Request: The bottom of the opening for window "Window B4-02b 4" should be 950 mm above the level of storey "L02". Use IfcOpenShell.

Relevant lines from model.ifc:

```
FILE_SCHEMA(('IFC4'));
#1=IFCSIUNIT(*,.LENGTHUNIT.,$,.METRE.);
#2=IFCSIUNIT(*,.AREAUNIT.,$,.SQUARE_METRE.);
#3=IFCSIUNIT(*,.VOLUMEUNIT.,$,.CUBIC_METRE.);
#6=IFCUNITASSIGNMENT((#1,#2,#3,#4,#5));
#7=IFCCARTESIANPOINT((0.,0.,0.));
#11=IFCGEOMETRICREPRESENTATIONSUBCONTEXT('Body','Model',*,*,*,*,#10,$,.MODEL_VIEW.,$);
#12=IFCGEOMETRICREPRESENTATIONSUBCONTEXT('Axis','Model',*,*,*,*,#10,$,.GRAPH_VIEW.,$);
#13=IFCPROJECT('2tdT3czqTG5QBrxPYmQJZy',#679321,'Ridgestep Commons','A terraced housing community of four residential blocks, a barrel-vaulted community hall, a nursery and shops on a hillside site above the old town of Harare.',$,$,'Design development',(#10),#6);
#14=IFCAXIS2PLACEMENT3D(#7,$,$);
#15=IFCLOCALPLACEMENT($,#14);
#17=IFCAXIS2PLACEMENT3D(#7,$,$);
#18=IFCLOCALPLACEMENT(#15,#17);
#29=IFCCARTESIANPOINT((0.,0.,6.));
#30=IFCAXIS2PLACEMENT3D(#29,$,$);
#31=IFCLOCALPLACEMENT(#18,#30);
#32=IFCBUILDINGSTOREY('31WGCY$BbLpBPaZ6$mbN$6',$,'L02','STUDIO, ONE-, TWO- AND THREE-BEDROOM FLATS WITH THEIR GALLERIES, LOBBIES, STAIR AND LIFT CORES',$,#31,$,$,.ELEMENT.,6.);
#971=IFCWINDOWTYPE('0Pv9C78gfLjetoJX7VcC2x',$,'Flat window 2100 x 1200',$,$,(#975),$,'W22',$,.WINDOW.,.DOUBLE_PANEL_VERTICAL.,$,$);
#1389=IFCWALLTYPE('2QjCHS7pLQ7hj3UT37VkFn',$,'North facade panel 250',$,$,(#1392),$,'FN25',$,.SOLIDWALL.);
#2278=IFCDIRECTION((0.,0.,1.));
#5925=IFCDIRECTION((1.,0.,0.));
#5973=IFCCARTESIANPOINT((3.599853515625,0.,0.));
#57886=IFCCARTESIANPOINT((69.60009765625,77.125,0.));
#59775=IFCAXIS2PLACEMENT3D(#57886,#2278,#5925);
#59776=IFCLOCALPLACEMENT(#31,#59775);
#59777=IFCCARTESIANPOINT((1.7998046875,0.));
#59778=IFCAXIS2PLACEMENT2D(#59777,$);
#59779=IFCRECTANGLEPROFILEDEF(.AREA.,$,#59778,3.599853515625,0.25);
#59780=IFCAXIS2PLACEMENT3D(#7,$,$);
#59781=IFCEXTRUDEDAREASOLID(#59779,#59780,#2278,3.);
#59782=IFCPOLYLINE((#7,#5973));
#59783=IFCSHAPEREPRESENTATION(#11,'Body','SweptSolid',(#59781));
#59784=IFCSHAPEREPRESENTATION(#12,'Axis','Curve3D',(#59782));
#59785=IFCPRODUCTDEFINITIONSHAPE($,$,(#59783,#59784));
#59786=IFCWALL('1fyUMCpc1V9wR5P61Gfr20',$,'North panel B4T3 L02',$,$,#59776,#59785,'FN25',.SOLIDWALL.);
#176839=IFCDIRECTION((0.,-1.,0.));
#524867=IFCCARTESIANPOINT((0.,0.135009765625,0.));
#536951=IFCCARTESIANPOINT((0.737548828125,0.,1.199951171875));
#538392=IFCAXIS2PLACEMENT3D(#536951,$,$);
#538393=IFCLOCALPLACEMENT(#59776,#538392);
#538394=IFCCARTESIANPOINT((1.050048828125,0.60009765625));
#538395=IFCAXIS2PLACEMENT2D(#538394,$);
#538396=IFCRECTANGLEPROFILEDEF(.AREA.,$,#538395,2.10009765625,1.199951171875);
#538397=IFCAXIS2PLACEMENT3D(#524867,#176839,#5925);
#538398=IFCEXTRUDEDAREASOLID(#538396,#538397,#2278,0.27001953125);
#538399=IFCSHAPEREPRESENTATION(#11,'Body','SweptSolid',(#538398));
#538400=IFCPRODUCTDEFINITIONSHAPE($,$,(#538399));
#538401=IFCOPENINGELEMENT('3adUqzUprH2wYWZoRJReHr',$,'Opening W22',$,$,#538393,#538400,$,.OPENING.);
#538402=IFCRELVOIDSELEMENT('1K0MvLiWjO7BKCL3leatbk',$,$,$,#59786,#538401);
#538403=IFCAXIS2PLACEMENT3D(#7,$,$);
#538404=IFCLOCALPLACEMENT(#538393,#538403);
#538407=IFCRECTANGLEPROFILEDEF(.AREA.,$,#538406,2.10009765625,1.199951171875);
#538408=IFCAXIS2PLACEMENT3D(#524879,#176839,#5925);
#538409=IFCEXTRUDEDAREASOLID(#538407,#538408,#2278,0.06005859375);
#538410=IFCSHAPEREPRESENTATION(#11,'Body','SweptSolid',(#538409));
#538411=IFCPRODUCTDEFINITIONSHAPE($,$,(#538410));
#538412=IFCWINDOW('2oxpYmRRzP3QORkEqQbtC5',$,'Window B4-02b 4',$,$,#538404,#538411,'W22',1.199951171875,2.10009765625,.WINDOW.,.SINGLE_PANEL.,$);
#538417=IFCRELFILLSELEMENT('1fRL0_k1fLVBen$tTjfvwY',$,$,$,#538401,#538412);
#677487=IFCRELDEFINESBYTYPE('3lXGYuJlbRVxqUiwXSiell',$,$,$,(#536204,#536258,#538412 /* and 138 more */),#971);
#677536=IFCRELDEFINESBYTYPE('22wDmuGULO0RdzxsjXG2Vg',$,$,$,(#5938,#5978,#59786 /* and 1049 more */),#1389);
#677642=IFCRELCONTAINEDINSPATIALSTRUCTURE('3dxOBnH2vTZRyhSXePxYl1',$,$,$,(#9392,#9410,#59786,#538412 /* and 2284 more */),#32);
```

```python
import numpy as np
import ifcopenshell
import ifcopenshell.api.geometry
import ifcopenshell.geom
import ifcopenshell.util.element
import ifcopenshell.util.placement
import ifcopenshell.util.shape
import ifcopenshell.util.unit

model = ifcopenshell.open("model.ifc")
unit_scale = ifcopenshell.util.unit.calculate_unit_scale(model)

window = model.by_guid("2oxpYmRRzP3QORkEqQbtC5")
opening = window.FillsVoids[0].RelatingOpeningElement
storey = ifcopenshell.util.element.get_container(window, ifc_class="IfcBuildingStorey")
level = ifcopenshell.util.placement.get_local_placement(storey.ObjectPlacement)[2, 3]

# The opening's origin need not be at the sill, so measure its lowest point.
shape = ifcopenshell.geom.create_shape(ifcopenshell.geom.settings(), opening)
bottom = ifcopenshell.util.shape.get_shape_bottom_elevation(shape, shape.geometry) / unit_scale
dz = level + 0.95 / unit_scale - bottom

shift = np.array([0.0, 0.0, dz])
# The window is placed relative to its opening, so it follows when the opening moves.
matrix = ifcopenshell.util.placement.get_local_placement(opening.ObjectPlacement)
matrix[:3, 3] += shift
ifcopenshell.api.geometry.edit_object_placement(
    model, product=opening, matrix=matrix, is_si=False, should_transform_children=True
)

print(f"moved by {dz * unit_scale:+.3f} m")

model.write("model_rev.ifc")
```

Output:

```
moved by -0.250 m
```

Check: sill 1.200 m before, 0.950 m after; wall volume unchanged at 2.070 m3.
